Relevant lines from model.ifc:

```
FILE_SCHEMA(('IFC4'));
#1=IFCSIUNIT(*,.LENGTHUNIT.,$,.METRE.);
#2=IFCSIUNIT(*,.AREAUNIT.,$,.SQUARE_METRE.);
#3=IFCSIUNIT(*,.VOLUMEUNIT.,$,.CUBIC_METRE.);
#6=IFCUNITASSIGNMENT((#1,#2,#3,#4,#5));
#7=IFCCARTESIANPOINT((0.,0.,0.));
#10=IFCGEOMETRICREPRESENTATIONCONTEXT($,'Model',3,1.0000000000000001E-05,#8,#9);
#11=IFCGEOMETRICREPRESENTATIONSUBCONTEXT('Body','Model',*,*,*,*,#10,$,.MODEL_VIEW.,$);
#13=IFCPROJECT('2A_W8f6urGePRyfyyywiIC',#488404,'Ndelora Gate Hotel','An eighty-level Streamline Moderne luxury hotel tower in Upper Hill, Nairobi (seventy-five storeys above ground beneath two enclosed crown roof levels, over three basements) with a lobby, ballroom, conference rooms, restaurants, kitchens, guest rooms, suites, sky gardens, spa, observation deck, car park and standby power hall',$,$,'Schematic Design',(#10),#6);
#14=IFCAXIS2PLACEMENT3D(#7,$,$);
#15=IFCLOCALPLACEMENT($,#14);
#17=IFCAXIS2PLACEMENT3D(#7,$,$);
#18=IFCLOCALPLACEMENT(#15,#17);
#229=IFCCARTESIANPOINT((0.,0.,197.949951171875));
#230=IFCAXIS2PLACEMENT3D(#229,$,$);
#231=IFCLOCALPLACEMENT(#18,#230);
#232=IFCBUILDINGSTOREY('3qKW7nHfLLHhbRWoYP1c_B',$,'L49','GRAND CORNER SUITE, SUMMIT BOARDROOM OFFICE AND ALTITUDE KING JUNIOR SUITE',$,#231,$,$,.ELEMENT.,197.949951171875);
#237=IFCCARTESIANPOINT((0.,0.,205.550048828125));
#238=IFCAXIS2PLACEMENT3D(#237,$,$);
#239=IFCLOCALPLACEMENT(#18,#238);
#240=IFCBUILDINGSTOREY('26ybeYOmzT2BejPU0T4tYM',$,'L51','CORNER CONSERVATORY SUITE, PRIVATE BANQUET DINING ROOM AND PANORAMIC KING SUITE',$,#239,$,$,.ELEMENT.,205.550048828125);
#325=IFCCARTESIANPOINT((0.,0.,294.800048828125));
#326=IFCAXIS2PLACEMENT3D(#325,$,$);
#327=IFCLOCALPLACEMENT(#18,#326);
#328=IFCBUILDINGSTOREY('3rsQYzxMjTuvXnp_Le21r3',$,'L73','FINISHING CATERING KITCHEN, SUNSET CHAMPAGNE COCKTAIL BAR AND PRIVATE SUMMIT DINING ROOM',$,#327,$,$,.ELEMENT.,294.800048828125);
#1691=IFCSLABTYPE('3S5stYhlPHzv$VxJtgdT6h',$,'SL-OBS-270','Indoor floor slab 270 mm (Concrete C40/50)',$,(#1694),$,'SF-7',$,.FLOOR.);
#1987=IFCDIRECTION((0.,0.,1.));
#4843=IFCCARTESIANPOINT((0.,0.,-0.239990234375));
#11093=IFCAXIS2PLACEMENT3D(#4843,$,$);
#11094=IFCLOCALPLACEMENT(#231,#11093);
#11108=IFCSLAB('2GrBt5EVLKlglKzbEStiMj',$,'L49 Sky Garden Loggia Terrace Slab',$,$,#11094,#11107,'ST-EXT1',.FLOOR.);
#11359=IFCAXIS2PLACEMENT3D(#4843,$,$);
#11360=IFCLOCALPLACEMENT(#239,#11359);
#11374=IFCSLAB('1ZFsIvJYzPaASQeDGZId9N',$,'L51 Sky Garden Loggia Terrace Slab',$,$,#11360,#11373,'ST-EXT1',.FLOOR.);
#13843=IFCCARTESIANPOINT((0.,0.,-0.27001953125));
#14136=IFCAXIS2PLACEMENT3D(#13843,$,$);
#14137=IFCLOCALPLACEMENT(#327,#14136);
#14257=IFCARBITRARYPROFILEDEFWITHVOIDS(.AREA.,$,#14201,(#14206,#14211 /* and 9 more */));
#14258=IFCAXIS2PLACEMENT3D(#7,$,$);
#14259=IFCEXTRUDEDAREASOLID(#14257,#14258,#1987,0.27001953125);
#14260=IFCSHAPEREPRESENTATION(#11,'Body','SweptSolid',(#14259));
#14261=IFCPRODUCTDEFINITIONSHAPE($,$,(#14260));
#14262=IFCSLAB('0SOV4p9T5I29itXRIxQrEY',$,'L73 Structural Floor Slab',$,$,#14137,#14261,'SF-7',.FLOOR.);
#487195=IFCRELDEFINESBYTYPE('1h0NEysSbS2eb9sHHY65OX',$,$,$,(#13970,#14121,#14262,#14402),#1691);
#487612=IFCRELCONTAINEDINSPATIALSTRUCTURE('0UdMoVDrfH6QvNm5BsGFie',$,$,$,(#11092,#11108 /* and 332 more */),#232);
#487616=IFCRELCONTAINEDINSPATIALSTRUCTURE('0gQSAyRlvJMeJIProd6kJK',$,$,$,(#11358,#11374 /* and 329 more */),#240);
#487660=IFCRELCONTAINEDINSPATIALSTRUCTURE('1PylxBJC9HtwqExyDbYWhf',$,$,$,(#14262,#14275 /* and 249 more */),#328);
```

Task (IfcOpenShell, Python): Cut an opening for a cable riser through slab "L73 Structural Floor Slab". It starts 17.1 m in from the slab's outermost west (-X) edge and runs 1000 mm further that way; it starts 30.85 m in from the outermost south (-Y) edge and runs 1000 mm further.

```python
import numpy as np
import ifcopenshell
import ifcopenshell.api.feature
import ifcopenshell.api.geometry
import ifcopenshell.api.root
import ifcopenshell.geom
import ifcopenshell.util.placement
import ifcopenshell.util.representation
import ifcopenshell.util.shape
import ifcopenshell.util.unit

model = ifcopenshell.open("model.ifc")
unit_scale = ifcopenshell.util.unit.calculate_unit_scale(model)
settings = ifcopenshell.geom.settings()


def volume(element):
    """Net volume in cubic metres, openings subtracted."""
    shape = ifcopenshell.geom.create_shape(settings, element)
    return ifcopenshell.util.shape.get_volume(shape.geometry)


slab = model.by_id(14262)
before = volume(slab)

# Extent in the slab's own axes, in metres. The edges named are its -X and -Y sides.
slab_shape = ifcopenshell.geom.create_shape(settings, slab)
vertices = ifcopenshell.util.shape.get_vertices(slab_shape.geometry)
x_min, y_min, bottom = vertices.min(axis=0)
top = vertices[:, 2].max()

opening = ifcopenshell.api.root.create_entity(model, ifc_class="IfcOpeningElement", name="Cable riser opening", predefined_type="OPENING")
context = ifcopenshell.util.representation.get_context(model, "Model", "Body", "MODEL_VIEW")
width, depth = 1, 1
outline = [(0.0, 0.0), (width, 0.0), (width, depth), (0.0, depth), (0.0, 0.0)]
# Overshoot both faces by 50 mm so the cut is clean.
shape = ifcopenshell.api.geometry.add_slab_representation(
    model, context=context, depth=top - bottom + 0.1, polyline=outline
)
ifcopenshell.api.geometry.assign_representation(model, product=opening, representation=shape)

matrix = ifcopenshell.util.placement.get_local_placement(slab.ObjectPlacement)
matrix[:, 3] = matrix @ np.append(np.array([x_min + 17.1, y_min + 30.85, bottom - 0.05]) / unit_scale, 1.0)
ifcopenshell.api.geometry.edit_object_placement(model, product=opening, matrix=matrix, is_si=False)
ifcopenshell.api.feature.add_feature(model, feature=opening, element=slab)

after = volume(slab)

print(f"slab volume {before:.3f} -> {after:.3f} m3")

model.write("model_rev.ifc")
```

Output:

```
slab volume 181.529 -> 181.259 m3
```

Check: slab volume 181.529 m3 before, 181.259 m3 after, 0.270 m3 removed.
